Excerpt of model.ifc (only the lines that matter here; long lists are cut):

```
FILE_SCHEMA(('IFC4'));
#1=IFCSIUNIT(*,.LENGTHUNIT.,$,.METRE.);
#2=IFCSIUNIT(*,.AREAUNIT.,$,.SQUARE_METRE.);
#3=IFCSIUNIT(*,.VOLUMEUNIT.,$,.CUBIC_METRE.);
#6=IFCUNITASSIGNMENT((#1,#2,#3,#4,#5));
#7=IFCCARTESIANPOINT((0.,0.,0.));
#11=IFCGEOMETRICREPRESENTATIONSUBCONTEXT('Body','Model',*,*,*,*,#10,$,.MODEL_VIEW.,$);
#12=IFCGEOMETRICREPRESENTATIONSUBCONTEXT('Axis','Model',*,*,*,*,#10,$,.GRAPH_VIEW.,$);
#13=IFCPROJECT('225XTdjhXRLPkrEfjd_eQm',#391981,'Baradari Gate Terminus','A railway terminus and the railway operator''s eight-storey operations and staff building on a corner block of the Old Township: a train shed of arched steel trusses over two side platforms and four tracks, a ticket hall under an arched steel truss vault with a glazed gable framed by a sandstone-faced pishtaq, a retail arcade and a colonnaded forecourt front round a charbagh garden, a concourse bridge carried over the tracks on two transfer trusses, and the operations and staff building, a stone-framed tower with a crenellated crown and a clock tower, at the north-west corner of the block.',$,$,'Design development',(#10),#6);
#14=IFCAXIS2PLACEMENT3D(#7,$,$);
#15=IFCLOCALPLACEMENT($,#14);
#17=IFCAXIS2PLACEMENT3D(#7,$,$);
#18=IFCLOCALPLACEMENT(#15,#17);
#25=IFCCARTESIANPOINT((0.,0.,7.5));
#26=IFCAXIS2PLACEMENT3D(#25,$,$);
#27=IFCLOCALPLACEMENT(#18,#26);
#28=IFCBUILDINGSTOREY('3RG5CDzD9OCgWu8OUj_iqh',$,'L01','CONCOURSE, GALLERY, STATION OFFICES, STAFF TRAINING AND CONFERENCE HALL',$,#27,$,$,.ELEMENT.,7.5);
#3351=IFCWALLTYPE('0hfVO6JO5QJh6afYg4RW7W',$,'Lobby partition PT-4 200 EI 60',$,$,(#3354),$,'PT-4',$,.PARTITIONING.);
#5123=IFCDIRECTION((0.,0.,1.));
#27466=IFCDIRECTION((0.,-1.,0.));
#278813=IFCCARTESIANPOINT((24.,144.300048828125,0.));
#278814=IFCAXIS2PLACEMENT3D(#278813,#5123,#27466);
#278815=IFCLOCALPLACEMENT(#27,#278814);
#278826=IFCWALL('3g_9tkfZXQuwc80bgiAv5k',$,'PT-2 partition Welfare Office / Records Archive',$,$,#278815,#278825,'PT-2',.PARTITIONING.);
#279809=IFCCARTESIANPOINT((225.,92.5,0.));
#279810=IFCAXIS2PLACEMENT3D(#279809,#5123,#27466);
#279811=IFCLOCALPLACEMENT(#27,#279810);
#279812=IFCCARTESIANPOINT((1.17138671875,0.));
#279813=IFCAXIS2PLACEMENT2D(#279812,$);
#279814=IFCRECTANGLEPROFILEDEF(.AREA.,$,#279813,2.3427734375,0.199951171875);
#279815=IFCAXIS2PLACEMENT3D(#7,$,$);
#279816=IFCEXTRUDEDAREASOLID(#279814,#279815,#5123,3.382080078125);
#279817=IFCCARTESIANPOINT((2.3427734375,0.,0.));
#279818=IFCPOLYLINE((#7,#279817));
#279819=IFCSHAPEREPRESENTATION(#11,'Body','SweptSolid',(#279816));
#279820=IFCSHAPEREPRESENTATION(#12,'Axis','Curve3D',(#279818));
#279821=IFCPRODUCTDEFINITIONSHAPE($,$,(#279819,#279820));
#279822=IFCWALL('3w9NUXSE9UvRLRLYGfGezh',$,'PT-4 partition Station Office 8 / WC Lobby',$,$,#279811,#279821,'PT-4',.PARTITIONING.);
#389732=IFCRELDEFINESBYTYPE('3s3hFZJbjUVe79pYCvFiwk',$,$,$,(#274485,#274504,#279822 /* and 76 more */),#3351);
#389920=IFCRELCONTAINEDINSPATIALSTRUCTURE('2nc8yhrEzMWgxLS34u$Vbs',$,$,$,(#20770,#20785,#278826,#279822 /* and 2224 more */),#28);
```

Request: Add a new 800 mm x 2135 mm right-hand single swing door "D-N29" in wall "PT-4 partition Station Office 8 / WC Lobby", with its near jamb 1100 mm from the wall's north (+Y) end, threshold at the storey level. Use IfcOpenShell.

```python
import numpy as np
import ifcopenshell
import ifcopenshell.api.feature
import ifcopenshell.api.geometry
import ifcopenshell.api.root
import ifcopenshell.api.spatial
import ifcopenshell.geom
import ifcopenshell.util.element
import ifcopenshell.util.placement
import ifcopenshell.util.representation
import ifcopenshell.util.shape
import ifcopenshell.util.unit

model = ifcopenshell.open("model.ifc")
unit_scale = ifcopenshell.util.unit.calculate_unit_scale(model)
settings = ifcopenshell.geom.settings()


def volume(element):
    """Net volume in cubic metres, openings subtracted."""
    shape = ifcopenshell.geom.create_shape(settings, element)
    return ifcopenshell.util.shape.get_volume(shape.geometry)


wall = model.by_guid("3w9NUXSE9UvRLRLYGfGezh")
storey = ifcopenshell.util.element.get_container(wall, ifc_class="IfcBuildingStorey")
context = ifcopenshell.util.representation.get_context(model, "Model", "Body", "MODEL_VIEW")
before = volume(wall)

width, height, from_end, sill = 0.8, 2.135, 1.1, 0.0  # metres

# The wall runs along its own X axis, and the end named is its -X end.
wall_shape = ifcopenshell.geom.create_shape(settings, wall)
x, y, z = ifcopenshell.util.shape.get_vertices(wall_shape.geometry).T
start = x.min() + from_end
face, thickness = float(y.min()), float(y.max() - y.min())
wall_matrix = ifcopenshell.util.placement.get_local_placement(wall.ObjectPlacement)
level = ifcopenshell.util.placement.get_local_placement(storey.ObjectPlacement)[2, 3]


def in_wall(x, y):
    """Placement at x, y metres in the wall's axes, at sill height."""
    matrix = wall_matrix.copy()
    matrix[:, 3] = wall_matrix @ np.array([x / unit_scale, y / unit_scale, 0.0, 1.0])
    matrix[2, 3] = level + sill / unit_scale
    return matrix


# Opening: a box that overshoots both wall faces by 50 mm.
opening = ifcopenshell.api.root.create_entity(model, ifc_class="IfcOpeningElement", predefined_type="OPENING")
box = ifcopenshell.api.geometry.add_wall_representation(
    model, context=context, length=width, height=height, thickness=thickness + 0.1
)
ifcopenshell.api.geometry.assign_representation(model, product=opening, representation=box)
ifcopenshell.api.geometry.edit_object_placement(model, product=opening, matrix=in_wall(start, face - 0.05), is_si=False)
ifcopenshell.api.feature.add_feature(model, feature=opening, element=wall)

door = ifcopenshell.api.root.create_entity(model, ifc_class="IfcDoor", name="D-N29", predefined_type="DOOR")
door.OverallWidth, door.OverallHeight = width / unit_scale, height / unit_scale
door.OperationType = "SINGLE_SWING_RIGHT"
body = ifcopenshell.api.geometry.add_door_representation(
    model,
    context=context,
    overall_width=door.OverallWidth,
    overall_height=door.OverallHeight,
    operation_type="SINGLE_SWING_RIGHT",
    lining_properties={"LiningDepth": thickness / unit_scale, "ThresholdDepth": thickness / unit_scale},
)
ifcopenshell.api.geometry.assign_representation(model, product=door, representation=body)
ifcopenshell.api.spatial.assign_container(model, products=[door], relating_structure=storey)
ifcopenshell.api.feature.add_filling(model, opening=opening, element=door)

# The lining spans the wall, so the door starts at the wall face.
ifcopenshell.api.geometry.edit_object_placement(model, product=door, matrix=in_wall(start, face), is_si=False)

after = volume(wall)

print(f"wall volume {before:.3f} -> {after:.3f} m3")

model.write("model_v2.ifc")
```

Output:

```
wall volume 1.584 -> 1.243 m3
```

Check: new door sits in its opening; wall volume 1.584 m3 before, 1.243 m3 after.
